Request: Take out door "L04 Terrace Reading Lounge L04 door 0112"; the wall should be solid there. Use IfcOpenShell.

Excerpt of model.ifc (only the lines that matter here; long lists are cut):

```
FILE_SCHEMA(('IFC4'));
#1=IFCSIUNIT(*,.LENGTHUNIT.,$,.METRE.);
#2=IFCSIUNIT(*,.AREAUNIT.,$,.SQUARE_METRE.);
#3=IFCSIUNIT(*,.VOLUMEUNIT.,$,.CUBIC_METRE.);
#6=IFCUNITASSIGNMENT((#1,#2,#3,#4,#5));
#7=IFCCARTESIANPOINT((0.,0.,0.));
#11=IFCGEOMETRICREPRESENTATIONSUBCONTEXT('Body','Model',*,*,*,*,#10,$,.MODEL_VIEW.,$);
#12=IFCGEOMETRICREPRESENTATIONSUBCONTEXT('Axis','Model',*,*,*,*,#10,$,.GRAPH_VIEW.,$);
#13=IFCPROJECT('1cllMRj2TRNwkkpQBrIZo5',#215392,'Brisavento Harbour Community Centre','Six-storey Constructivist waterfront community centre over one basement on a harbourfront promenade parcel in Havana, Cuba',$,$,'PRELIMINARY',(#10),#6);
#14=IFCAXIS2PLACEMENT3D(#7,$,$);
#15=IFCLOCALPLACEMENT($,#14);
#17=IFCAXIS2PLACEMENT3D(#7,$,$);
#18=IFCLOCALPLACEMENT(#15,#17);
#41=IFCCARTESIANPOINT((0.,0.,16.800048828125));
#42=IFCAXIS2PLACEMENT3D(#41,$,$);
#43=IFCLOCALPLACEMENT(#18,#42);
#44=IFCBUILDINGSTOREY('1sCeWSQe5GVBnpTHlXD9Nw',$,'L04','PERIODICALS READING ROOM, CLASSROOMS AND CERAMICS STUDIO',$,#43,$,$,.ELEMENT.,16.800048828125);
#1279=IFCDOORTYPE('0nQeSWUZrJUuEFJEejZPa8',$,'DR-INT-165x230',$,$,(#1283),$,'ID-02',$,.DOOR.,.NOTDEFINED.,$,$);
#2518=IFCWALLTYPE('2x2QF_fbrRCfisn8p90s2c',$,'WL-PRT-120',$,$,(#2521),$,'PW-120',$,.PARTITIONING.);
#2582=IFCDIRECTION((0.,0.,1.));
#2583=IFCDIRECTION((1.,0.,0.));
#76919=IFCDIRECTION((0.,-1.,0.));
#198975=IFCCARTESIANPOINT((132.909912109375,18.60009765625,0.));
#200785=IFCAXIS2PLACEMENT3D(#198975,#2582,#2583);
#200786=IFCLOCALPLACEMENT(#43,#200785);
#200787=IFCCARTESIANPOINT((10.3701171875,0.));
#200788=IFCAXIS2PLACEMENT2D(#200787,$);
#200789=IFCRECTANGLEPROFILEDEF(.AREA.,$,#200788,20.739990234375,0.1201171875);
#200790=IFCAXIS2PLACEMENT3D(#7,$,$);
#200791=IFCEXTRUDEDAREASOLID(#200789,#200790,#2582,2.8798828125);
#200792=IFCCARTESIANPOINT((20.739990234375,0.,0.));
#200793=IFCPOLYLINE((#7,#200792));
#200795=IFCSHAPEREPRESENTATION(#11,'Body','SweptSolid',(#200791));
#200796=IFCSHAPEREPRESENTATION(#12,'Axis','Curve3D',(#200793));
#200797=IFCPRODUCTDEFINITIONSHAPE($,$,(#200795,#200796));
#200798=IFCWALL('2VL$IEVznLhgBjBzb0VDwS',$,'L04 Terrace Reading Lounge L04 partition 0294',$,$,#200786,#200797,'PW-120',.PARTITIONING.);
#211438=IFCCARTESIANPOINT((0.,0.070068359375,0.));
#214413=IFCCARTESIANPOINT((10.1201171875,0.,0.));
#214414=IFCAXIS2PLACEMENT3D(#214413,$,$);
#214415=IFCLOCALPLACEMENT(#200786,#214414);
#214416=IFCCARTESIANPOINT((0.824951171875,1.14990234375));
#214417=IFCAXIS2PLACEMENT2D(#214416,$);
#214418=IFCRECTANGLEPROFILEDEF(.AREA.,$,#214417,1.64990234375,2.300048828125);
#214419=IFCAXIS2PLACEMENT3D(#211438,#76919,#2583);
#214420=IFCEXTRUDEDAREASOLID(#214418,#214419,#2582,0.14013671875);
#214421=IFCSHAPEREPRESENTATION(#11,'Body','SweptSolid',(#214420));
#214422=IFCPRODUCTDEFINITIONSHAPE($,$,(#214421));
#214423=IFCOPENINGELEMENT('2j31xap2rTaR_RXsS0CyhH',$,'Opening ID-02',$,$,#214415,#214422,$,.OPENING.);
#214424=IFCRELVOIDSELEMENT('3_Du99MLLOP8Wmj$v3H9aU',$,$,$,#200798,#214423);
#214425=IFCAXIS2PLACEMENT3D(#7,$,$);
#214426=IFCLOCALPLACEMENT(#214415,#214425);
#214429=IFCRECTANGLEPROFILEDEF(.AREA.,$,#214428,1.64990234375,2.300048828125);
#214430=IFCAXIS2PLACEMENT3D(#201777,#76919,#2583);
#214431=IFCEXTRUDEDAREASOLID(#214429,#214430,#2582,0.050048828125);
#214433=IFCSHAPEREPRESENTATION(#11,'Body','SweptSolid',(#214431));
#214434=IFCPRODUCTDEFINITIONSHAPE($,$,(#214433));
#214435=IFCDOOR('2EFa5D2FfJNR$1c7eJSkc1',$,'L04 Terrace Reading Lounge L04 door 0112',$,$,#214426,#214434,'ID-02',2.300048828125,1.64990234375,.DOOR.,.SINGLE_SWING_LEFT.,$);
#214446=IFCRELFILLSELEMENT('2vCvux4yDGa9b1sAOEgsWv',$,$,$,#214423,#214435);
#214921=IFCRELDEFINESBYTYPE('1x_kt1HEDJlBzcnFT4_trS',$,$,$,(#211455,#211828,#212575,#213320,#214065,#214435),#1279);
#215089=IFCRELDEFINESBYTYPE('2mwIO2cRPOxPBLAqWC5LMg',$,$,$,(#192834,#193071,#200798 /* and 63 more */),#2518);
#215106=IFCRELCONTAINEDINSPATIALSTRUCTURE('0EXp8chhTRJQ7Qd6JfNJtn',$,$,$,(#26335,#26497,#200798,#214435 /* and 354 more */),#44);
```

```python
import ifcopenshell
import ifcopenshell.api.feature
import ifcopenshell.api.root
import ifcopenshell.geom
import ifcopenshell.util.shape

model = ifcopenshell.open("model.ifc")
settings = ifcopenshell.geom.settings()


def volume(element):
    """Net volume in cubic metres, openings subtracted."""
    shape = ifcopenshell.geom.create_shape(settings, element)
    return ifcopenshell.util.shape.get_volume(shape.geometry)


door = model.by_guid("2EFa5D2FfJNR$1c7eJSkc1")
opening = door.FillsVoids[0].RelatingOpeningElement
wall = opening.VoidsElements[0].RelatingBuildingElement
before = volume(wall)

ifcopenshell.api.root.remove_product(model, product=door)
ifcopenshell.api.feature.remove_feature(model, feature=opening)

after = volume(wall)

print(f"wall volume {before:.3f} -> {after:.3f} m3")

model.write("model_edited.ifc")
```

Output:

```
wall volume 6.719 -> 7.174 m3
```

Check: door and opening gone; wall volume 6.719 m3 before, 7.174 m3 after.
